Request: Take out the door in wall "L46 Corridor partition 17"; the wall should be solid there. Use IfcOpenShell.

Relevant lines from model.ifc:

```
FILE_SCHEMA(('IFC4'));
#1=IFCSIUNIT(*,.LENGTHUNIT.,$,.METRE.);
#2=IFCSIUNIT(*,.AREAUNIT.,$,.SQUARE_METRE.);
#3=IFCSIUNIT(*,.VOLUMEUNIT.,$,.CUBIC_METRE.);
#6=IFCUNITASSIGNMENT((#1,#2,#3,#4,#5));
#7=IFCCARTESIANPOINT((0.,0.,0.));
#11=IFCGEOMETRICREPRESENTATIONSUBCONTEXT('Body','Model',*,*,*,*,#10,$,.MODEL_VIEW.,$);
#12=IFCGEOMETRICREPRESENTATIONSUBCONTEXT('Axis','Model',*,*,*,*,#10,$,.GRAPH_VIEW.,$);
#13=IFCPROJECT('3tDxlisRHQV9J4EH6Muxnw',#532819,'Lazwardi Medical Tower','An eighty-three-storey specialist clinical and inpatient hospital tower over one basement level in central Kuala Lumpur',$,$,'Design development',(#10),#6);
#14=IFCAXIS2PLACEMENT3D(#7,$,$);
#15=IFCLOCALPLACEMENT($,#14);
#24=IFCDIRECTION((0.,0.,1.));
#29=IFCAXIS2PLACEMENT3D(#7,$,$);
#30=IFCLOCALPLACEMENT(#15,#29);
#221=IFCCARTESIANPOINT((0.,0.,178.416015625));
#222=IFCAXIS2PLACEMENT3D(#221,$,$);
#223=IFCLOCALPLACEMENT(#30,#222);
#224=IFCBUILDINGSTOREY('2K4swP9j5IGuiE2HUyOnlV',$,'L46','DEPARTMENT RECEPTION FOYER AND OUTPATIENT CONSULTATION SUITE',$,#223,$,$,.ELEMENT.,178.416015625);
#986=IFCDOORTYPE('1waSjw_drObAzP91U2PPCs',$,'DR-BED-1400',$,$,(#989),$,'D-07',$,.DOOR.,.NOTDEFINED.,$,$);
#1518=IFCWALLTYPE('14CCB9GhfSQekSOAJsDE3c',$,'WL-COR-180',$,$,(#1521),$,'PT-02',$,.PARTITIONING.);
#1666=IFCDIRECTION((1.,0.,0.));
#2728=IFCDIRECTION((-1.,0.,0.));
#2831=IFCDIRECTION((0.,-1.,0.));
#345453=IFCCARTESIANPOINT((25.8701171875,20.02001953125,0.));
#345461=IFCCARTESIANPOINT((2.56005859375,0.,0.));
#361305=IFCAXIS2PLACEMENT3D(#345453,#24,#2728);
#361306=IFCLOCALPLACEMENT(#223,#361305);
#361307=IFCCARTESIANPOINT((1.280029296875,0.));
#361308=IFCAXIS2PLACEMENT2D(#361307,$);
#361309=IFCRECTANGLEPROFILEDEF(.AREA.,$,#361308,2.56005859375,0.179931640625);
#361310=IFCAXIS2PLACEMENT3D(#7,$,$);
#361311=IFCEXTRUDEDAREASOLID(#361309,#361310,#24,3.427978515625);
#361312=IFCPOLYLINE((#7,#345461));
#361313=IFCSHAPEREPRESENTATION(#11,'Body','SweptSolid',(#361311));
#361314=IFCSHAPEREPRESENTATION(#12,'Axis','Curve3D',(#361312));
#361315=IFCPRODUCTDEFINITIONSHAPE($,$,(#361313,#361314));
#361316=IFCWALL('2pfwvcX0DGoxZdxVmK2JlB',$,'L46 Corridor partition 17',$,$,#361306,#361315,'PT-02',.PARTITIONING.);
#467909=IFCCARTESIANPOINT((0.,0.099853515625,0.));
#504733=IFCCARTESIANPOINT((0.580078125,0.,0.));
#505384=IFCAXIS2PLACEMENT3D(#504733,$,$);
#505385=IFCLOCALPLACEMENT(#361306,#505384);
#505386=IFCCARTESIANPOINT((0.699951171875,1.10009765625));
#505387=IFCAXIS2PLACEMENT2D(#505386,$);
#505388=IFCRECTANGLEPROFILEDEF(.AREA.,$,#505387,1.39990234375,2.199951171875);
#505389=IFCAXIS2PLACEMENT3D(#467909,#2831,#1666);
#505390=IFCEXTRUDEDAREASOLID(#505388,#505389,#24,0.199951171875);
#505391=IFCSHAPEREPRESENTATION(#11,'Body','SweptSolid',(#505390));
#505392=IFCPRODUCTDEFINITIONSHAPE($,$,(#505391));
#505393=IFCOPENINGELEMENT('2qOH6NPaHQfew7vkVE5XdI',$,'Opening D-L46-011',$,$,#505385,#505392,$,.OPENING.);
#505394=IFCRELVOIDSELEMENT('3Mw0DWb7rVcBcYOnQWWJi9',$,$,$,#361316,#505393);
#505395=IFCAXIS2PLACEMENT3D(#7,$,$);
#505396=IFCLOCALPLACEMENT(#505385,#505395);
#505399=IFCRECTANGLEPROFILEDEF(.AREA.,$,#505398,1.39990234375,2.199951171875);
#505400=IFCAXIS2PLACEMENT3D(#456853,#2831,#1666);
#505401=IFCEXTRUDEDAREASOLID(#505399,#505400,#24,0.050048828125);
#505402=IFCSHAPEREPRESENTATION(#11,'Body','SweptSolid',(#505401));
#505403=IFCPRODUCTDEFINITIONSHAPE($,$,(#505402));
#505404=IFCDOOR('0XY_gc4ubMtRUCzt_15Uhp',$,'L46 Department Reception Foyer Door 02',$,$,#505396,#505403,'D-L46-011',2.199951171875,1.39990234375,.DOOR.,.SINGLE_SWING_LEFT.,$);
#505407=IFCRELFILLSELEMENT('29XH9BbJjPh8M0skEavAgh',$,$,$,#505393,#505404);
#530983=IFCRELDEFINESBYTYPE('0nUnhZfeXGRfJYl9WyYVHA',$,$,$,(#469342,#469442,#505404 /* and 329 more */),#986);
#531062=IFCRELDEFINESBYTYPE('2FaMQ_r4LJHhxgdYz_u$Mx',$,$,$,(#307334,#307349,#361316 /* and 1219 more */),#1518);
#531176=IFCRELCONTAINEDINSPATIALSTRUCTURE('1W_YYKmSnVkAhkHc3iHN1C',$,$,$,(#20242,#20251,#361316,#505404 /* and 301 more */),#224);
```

```python
import ifcopenshell
import ifcopenshell.api.feature
import ifcopenshell.api.root
import ifcopenshell.geom
import ifcopenshell.util.shape

model = ifcopenshell.open("model.ifc")
settings = ifcopenshell.geom.settings()


def volume(element):
    """Net volume in cubic metres, openings subtracted."""
    shape = ifcopenshell.geom.create_shape(settings, element)
    return ifcopenshell.util.shape.get_volume(shape.geometry)


door = model.by_guid("0XY_gc4ubMtRUCzt_15Uhp")
opening = door.FillsVoids[0].RelatingOpeningElement
wall = opening.VoidsElements[0].RelatingBuildingElement
before = volume(wall)

ifcopenshell.api.root.remove_product(model, product=door)
ifcopenshell.api.feature.remove_feature(model, feature=opening)

after = volume(wall)

print(f"wall volume {before:.3f} -> {after:.3f} m3")

model.write("model_edited.ifc")
```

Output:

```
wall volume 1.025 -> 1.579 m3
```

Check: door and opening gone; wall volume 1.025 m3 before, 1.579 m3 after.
